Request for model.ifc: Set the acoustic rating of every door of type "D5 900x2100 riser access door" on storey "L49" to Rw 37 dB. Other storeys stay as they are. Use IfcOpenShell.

First a look at what the model holds.

```python
import ifcopenshell
import ifcopenshell.util.element

model = ifcopenshell.open("model.ifc")
print(model.schema)
storey = next(s for s in model.by_type("IfcBuildingStorey") if s.Name == "L49")
doors = [e for e in ifcopenshell.util.element.get_decomposition(storey) if e.is_a("IfcDoor")]
seen = {}
for e in doors:
    element_type = ifcopenshell.util.element.get_type(e)
    key = (element_type.Name if element_type != e and element_type else None, ifcopenshell.util.element.get_pset(e, "Pset_DoorCommon", "AcousticRating"))
    seen[key] = seen.get(key, 0) + 1
for (name, value), count in sorted(seen.items(), key=str):
    print(count, "x", name, "|", value)
```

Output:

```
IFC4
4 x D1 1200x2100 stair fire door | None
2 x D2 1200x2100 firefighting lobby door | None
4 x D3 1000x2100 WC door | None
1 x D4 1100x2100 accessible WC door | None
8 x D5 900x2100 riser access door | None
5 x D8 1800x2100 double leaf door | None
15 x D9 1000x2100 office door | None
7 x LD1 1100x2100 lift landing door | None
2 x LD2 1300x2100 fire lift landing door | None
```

```python
import ifcopenshell
import ifcopenshell.api.pset
import ifcopenshell.util.element

model = ifcopenshell.open("model.ifc")

storey = next(s for s in model.by_type("IfcBuildingStorey") if s.Name == "L49")
doors = [e for e in ifcopenshell.util.element.get_decomposition(storey) if e.is_a("IfcDoor")]

count = 0
for e in doors:
    element_type = ifcopenshell.util.element.get_type(e)
    if element_type in (None, e) or element_type.Name != "D5 900x2100 riser access door":
        continue
    found = ifcopenshell.util.element.get_pset(e, "Pset_DoorCommon", should_inherit=False)
    if found:
        pset = model.by_id(found["id"])
        if len(ifcopenshell.util.element.get_elements_by_pset(pset)) > 1:
            pset = ifcopenshell.api.pset.unshare_pset(model, products=[e], pset=pset)[0]
    else:
        pset = ifcopenshell.api.pset.add_pset(model, product=e, name="Pset_DoorCommon")
    ifcopenshell.api.pset.edit_pset(model, pset=pset, properties={"AcousticRating": "Rw 37 dB"})
    count += 1

print(count, "doors updated")

model.write("model_v2.ifc")
```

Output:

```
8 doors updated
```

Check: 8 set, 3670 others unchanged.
